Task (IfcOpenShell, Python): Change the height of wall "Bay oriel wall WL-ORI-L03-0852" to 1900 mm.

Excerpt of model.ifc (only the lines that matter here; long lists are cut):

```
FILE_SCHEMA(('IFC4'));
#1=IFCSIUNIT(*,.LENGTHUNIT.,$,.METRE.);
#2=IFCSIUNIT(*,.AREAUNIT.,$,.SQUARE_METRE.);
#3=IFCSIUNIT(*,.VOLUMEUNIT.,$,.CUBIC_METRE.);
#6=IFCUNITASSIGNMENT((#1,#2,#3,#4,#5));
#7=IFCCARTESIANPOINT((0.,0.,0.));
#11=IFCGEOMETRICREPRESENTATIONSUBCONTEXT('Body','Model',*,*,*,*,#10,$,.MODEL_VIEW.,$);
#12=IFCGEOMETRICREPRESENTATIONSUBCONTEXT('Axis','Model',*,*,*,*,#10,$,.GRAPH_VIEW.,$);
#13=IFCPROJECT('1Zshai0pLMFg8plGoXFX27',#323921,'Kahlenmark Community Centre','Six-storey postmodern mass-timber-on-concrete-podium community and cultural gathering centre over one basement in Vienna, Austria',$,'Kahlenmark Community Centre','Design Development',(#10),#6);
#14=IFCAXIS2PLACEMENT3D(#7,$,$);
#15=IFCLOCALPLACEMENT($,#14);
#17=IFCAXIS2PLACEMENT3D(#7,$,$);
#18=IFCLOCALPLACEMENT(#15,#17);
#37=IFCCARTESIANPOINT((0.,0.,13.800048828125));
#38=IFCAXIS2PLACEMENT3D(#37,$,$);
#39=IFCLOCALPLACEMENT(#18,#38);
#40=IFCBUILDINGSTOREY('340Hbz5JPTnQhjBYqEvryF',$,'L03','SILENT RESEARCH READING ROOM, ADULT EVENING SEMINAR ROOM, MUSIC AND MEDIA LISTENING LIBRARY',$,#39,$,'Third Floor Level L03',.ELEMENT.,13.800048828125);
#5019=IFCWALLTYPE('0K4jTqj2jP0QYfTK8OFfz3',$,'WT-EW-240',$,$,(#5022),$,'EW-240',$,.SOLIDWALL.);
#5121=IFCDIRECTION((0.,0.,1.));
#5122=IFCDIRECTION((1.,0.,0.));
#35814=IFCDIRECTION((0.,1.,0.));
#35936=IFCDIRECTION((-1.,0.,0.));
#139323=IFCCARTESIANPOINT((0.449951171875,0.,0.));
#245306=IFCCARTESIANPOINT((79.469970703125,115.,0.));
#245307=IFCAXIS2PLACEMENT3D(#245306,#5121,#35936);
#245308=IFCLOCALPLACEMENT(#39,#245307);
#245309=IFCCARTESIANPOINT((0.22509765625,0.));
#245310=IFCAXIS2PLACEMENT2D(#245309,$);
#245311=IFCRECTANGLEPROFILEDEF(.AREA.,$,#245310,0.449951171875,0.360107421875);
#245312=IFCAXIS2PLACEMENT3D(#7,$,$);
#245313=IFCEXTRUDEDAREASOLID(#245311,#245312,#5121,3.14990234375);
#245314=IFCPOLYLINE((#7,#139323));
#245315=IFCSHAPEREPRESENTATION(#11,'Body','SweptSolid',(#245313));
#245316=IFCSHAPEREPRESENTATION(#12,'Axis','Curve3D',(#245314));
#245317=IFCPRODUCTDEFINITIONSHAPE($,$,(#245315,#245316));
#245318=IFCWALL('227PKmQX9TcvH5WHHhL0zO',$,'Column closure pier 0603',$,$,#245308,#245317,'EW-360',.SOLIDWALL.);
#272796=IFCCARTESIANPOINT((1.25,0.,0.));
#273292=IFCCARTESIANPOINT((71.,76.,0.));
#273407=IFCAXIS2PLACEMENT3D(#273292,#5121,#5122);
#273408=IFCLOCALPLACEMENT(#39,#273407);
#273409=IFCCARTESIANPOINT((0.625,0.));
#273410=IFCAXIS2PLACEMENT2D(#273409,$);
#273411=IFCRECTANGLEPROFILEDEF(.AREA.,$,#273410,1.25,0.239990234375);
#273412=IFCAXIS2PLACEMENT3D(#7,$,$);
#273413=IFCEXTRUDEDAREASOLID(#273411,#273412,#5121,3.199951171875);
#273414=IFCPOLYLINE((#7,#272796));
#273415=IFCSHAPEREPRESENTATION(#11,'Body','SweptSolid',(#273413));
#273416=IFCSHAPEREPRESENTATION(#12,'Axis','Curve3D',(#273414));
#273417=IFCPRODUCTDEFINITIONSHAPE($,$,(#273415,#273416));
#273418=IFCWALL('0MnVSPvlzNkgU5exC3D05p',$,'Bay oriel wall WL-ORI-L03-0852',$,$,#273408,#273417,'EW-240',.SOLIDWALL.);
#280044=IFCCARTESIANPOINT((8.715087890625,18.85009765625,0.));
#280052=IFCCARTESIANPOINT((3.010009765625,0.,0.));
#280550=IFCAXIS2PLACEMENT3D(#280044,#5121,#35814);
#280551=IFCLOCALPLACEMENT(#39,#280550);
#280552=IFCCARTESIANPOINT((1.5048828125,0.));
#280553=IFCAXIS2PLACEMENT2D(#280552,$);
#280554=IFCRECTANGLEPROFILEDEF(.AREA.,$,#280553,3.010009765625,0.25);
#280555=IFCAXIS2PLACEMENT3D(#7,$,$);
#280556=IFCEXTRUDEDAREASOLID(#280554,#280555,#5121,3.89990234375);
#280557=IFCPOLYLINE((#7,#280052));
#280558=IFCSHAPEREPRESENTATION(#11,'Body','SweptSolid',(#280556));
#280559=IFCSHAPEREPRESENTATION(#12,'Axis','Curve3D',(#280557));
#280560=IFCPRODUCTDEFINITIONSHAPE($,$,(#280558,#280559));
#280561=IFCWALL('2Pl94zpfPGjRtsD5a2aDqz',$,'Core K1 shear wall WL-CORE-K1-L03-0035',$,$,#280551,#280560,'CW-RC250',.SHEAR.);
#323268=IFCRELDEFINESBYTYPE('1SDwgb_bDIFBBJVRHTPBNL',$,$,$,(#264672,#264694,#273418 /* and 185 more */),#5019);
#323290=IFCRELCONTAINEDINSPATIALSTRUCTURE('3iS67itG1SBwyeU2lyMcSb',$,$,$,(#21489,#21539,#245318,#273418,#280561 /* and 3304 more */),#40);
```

```python
import ifcopenshell
import ifcopenshell.geom
import ifcopenshell.util.representation
import ifcopenshell.util.shape
import ifcopenshell.util.unit

model = ifcopenshell.open("model.ifc")
unit_scale = ifcopenshell.util.unit.calculate_unit_scale(model)
settings = ifcopenshell.geom.settings()


def volume(element):
    """Net volume in cubic metres, openings subtracted."""
    shape = ifcopenshell.geom.create_shape(settings, element)
    return ifcopenshell.util.shape.get_volume(shape.geometry)


wall = model.by_guid("0MnVSPvlzNkgU5exC3D05p")
before = volume(wall)

body = ifcopenshell.util.representation.get_representation(wall, "Model", "Body")
solid = body.Items[0]
old_height = solid.Depth
solid.Depth = 1.9 / unit_scale
after = volume(wall)

print(f"height {old_height:g} -> {solid.Depth:g}, volume {before:.3f} -> {after:.3f} m3")

model.write("model-out.ifc")
```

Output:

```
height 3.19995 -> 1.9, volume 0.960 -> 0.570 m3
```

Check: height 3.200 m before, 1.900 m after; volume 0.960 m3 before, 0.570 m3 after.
